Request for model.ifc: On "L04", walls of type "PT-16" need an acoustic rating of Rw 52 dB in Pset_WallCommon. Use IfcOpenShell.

First a look at what the model holds.

```python
import ifcopenshell
import ifcopenshell.util.element

model = ifcopenshell.open("model.ifc")
print(model.schema)
storey = next(s for s in model.by_type("IfcBuildingStorey") if s.Name == "L04")
walls = [e for e in ifcopenshell.util.element.get_decomposition(storey) if e.is_a("IfcWall")]
seen = {}
for e in walls:
    element_type = ifcopenshell.util.element.get_type(e)
    key = (element_type.Name if element_type != e and element_type else None, ifcopenshell.util.element.get_pset(e, "Pset_WallCommon", "AcousticRating"))
    seen[key] = seen.get(key, 0) + 1
for (name, value), count in sorted(seen.items(), key=str):
    print(count, "x", name, "|", value)
```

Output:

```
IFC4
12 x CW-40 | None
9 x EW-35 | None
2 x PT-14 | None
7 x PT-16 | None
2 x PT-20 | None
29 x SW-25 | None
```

```python
import ifcopenshell
import ifcopenshell.api.pset
import ifcopenshell.util.element

model = ifcopenshell.open("model.ifc")

storey = next(s for s in model.by_type("IfcBuildingStorey") if s.Name == "L04")
walls = [e for e in ifcopenshell.util.element.get_decomposition(storey) if e.is_a("IfcWall")]

count = 0
for e in walls:
    element_type = ifcopenshell.util.element.get_type(e)
    if element_type in (None, e) or element_type.Name != "PT-16":
        continue
    # add_pset returns the element's existing set when there is one.
    pset = ifcopenshell.api.pset.add_pset(model, product=e, name="Pset_WallCommon")
    ifcopenshell.api.pset.edit_pset(model, pset=pset, properties={"AcousticRating": "Rw 52 dB"})
    count += 1

print(count, "walls updated")

model.write("model_updated.ifc")
```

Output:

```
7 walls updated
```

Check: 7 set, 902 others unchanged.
